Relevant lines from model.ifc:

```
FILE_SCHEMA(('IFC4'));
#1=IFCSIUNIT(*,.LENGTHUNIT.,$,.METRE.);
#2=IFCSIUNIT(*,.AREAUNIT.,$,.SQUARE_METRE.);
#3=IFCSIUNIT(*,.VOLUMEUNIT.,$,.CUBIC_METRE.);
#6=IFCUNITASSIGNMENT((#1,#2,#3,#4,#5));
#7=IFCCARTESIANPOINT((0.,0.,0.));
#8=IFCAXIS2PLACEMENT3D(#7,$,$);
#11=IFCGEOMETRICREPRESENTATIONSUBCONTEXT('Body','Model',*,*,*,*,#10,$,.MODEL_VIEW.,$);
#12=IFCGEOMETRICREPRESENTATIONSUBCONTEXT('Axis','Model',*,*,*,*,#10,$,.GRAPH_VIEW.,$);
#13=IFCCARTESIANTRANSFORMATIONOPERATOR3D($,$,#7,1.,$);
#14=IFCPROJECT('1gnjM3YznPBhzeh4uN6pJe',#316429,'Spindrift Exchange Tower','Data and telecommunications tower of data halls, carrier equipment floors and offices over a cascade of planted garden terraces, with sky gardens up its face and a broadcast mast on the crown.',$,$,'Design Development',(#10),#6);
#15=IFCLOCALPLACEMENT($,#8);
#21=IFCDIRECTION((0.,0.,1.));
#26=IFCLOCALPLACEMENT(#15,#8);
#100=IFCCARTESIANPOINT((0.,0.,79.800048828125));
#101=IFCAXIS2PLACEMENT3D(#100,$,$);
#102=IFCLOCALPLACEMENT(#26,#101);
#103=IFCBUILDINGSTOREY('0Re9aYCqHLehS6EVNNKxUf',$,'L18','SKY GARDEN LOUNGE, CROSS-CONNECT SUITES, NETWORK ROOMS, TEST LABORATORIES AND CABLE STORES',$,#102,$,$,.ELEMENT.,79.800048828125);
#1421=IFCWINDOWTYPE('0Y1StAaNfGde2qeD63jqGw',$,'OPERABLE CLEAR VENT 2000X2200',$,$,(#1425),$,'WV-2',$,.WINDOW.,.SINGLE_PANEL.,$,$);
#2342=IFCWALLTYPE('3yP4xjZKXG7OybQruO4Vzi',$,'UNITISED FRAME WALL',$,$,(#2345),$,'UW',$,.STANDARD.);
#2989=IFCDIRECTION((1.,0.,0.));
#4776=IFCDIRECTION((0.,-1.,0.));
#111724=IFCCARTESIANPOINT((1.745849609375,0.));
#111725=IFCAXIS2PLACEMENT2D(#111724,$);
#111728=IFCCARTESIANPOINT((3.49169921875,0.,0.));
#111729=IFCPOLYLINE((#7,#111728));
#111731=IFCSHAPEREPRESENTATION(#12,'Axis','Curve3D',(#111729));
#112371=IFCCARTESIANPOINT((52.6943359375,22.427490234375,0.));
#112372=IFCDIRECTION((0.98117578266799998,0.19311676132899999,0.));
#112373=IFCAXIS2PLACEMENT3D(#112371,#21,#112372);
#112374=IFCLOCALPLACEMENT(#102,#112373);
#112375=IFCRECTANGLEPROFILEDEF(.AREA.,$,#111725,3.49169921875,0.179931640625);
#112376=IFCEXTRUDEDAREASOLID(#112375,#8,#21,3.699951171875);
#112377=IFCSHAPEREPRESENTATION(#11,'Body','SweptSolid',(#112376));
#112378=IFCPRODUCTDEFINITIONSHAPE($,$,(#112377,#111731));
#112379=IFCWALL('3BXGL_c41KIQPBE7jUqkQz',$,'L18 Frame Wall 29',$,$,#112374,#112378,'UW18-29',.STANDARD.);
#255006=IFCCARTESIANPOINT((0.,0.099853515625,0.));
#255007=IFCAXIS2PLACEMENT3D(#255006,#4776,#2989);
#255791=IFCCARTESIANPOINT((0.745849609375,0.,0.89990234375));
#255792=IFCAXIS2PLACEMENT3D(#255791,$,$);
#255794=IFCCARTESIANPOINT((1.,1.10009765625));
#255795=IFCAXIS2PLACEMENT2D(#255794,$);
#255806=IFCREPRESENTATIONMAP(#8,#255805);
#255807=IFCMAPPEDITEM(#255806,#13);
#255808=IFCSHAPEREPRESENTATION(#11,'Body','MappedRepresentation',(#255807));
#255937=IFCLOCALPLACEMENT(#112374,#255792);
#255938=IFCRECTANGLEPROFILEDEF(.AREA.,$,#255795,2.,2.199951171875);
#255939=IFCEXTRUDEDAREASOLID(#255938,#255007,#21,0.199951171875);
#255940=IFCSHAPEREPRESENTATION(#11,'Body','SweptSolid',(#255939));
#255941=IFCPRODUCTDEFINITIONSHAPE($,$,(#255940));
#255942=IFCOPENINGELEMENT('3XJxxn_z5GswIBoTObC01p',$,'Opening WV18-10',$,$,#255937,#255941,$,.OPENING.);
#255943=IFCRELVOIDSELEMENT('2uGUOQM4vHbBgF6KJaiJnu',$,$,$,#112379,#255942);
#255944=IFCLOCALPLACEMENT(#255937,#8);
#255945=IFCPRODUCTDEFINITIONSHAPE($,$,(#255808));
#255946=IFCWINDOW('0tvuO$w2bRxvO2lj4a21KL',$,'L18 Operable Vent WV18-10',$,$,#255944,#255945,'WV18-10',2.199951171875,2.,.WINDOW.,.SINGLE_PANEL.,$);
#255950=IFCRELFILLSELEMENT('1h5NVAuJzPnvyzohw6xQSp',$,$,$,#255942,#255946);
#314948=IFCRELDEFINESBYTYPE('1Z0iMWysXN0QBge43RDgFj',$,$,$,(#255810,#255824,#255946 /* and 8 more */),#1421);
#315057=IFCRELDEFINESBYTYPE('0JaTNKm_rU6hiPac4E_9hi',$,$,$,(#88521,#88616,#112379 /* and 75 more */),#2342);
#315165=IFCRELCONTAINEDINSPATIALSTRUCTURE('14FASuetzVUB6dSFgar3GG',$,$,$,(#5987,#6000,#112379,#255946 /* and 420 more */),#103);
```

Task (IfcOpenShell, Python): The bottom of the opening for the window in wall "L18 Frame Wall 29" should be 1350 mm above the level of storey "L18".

```python
import numpy as np
import ifcopenshell
import ifcopenshell.api.geometry
import ifcopenshell.geom
import ifcopenshell.util.element
import ifcopenshell.util.placement
import ifcopenshell.util.shape
import ifcopenshell.util.unit

model = ifcopenshell.open("model.ifc")
unit_scale = ifcopenshell.util.unit.calculate_unit_scale(model)

window = model.by_guid("0tvuO$w2bRxvO2lj4a21KL")
opening = window.FillsVoids[0].RelatingOpeningElement
storey = ifcopenshell.util.element.get_container(window, ifc_class="IfcBuildingStorey")
level = ifcopenshell.util.placement.get_local_placement(storey.ObjectPlacement)[2, 3]

# The opening's origin need not be at the sill, so measure its lowest point.
shape = ifcopenshell.geom.create_shape(ifcopenshell.geom.settings(), opening)
bottom = ifcopenshell.util.shape.get_shape_bottom_elevation(shape, shape.geometry) / unit_scale
dz = level + 1.35 / unit_scale - bottom

shift = np.array([0.0, 0.0, dz])
# The window is placed relative to its opening, so it follows when the opening moves.
matrix = ifcopenshell.util.placement.get_local_placement(opening.ObjectPlacement)
matrix[:3, 3] += shift
ifcopenshell.api.geometry.edit_object_placement(
    model, product=opening, matrix=matrix, is_si=False, should_transform_children=True
)

print(f"moved by {dz * unit_scale:+.3f} m")

model.write("model_edited.ifc")
```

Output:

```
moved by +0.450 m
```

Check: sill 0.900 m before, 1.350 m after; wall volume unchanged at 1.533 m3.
